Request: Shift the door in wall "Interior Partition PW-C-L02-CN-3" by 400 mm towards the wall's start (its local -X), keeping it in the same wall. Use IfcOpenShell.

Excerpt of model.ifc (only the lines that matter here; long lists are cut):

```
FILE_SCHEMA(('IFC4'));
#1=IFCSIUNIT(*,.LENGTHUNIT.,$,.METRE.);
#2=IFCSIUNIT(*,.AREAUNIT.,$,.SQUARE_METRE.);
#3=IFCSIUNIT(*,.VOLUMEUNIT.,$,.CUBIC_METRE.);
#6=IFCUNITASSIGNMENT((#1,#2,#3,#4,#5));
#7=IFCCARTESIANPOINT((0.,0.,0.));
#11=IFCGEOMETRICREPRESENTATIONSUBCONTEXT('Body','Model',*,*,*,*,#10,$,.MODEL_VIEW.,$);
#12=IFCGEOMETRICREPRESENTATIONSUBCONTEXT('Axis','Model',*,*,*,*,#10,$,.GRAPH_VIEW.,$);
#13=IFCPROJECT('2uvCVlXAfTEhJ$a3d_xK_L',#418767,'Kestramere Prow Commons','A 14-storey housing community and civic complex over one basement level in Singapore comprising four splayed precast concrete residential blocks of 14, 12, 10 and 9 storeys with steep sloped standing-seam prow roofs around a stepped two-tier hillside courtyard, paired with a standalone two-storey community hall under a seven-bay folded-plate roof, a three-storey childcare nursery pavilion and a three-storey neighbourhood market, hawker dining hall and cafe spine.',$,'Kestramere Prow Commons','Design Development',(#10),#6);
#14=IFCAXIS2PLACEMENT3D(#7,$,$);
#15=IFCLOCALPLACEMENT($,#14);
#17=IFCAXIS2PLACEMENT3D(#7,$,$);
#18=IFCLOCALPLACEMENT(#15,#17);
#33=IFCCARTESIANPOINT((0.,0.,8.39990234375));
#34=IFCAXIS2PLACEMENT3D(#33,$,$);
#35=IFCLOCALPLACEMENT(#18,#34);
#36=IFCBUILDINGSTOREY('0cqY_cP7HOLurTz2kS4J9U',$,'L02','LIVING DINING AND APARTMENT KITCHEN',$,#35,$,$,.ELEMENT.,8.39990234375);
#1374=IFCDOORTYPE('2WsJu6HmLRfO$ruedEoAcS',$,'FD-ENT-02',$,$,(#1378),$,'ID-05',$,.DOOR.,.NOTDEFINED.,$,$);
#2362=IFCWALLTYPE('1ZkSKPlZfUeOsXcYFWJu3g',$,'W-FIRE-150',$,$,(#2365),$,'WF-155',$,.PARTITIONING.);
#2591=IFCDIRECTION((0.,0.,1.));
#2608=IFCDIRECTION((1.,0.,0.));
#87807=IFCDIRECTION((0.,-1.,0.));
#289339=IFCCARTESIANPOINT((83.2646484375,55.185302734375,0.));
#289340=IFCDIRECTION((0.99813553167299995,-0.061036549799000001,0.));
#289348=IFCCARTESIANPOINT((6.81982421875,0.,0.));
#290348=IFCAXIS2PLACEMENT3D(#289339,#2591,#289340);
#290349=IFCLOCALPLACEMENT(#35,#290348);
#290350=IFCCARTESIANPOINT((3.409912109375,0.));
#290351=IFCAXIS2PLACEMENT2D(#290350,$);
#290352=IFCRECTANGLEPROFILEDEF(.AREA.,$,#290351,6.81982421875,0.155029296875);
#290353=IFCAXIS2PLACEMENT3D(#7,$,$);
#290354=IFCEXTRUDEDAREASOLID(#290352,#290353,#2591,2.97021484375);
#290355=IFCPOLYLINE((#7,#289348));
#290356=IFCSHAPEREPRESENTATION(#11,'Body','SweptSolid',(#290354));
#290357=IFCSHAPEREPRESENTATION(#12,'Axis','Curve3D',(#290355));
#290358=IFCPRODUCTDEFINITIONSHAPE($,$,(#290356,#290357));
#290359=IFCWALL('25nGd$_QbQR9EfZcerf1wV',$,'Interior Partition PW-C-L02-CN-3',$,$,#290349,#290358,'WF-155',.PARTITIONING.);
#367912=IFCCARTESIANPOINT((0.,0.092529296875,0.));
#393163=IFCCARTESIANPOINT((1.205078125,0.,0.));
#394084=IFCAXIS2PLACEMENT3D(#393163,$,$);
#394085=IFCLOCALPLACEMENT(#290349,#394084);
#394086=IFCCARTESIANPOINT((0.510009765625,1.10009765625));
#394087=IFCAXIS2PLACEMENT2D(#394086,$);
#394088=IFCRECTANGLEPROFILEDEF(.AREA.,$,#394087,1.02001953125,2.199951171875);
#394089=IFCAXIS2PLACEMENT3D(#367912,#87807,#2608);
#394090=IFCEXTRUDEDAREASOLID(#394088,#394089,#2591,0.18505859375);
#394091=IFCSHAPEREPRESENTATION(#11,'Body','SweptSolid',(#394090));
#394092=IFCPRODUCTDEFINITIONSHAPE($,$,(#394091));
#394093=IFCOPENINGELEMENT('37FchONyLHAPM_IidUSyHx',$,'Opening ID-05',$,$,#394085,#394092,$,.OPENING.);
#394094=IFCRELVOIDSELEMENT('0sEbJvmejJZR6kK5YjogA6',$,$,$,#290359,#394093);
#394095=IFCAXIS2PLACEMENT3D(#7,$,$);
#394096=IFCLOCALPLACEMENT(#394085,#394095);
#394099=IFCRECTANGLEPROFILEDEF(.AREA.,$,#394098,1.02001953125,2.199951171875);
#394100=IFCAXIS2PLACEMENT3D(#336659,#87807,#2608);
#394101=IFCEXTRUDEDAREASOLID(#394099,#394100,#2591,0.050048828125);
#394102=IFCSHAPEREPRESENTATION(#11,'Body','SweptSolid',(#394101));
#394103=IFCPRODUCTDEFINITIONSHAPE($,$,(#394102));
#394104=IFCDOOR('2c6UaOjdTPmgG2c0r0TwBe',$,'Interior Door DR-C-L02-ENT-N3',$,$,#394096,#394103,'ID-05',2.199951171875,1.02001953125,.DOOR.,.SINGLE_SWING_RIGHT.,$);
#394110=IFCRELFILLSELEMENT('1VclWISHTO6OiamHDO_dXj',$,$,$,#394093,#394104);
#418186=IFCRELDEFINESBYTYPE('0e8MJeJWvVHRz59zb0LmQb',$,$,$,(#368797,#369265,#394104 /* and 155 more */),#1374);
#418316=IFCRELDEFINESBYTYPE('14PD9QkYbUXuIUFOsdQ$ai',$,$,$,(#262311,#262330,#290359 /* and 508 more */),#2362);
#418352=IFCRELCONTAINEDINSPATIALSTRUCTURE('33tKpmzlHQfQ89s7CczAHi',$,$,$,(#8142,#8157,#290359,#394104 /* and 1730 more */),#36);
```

```python
import ifcopenshell
import ifcopenshell.api.geometry
import ifcopenshell.util.placement

model = ifcopenshell.open("model.ifc")

door = model.by_id(394104)
opening = door.FillsVoids[0].RelatingOpeningElement
wall = opening.VoidsElements[0].RelatingBuildingElement

wall_matrix = ifcopenshell.util.placement.get_local_placement(wall.ObjectPlacement)
shift = wall_matrix[:3, 0] * -0.4
before = ifcopenshell.util.placement.get_local_placement(door.ObjectPlacement)[:3, 3].copy()

# The door is placed relative to its opening, so it follows when the opening moves.
matrix = ifcopenshell.util.placement.get_local_placement(opening.ObjectPlacement)
matrix[:3, 3] += shift
ifcopenshell.api.geometry.edit_object_placement(
    model, product=opening, matrix=matrix, is_si=False, should_transform_children=True
)

after = ifcopenshell.util.placement.get_local_placement(door.ObjectPlacement)[:3, 3]
print("door moved by", (after - before).round(3) + 0.0)

model.write("model_v2.ifc")
```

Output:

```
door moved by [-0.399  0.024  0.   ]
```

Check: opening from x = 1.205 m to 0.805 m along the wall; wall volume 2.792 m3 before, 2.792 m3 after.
